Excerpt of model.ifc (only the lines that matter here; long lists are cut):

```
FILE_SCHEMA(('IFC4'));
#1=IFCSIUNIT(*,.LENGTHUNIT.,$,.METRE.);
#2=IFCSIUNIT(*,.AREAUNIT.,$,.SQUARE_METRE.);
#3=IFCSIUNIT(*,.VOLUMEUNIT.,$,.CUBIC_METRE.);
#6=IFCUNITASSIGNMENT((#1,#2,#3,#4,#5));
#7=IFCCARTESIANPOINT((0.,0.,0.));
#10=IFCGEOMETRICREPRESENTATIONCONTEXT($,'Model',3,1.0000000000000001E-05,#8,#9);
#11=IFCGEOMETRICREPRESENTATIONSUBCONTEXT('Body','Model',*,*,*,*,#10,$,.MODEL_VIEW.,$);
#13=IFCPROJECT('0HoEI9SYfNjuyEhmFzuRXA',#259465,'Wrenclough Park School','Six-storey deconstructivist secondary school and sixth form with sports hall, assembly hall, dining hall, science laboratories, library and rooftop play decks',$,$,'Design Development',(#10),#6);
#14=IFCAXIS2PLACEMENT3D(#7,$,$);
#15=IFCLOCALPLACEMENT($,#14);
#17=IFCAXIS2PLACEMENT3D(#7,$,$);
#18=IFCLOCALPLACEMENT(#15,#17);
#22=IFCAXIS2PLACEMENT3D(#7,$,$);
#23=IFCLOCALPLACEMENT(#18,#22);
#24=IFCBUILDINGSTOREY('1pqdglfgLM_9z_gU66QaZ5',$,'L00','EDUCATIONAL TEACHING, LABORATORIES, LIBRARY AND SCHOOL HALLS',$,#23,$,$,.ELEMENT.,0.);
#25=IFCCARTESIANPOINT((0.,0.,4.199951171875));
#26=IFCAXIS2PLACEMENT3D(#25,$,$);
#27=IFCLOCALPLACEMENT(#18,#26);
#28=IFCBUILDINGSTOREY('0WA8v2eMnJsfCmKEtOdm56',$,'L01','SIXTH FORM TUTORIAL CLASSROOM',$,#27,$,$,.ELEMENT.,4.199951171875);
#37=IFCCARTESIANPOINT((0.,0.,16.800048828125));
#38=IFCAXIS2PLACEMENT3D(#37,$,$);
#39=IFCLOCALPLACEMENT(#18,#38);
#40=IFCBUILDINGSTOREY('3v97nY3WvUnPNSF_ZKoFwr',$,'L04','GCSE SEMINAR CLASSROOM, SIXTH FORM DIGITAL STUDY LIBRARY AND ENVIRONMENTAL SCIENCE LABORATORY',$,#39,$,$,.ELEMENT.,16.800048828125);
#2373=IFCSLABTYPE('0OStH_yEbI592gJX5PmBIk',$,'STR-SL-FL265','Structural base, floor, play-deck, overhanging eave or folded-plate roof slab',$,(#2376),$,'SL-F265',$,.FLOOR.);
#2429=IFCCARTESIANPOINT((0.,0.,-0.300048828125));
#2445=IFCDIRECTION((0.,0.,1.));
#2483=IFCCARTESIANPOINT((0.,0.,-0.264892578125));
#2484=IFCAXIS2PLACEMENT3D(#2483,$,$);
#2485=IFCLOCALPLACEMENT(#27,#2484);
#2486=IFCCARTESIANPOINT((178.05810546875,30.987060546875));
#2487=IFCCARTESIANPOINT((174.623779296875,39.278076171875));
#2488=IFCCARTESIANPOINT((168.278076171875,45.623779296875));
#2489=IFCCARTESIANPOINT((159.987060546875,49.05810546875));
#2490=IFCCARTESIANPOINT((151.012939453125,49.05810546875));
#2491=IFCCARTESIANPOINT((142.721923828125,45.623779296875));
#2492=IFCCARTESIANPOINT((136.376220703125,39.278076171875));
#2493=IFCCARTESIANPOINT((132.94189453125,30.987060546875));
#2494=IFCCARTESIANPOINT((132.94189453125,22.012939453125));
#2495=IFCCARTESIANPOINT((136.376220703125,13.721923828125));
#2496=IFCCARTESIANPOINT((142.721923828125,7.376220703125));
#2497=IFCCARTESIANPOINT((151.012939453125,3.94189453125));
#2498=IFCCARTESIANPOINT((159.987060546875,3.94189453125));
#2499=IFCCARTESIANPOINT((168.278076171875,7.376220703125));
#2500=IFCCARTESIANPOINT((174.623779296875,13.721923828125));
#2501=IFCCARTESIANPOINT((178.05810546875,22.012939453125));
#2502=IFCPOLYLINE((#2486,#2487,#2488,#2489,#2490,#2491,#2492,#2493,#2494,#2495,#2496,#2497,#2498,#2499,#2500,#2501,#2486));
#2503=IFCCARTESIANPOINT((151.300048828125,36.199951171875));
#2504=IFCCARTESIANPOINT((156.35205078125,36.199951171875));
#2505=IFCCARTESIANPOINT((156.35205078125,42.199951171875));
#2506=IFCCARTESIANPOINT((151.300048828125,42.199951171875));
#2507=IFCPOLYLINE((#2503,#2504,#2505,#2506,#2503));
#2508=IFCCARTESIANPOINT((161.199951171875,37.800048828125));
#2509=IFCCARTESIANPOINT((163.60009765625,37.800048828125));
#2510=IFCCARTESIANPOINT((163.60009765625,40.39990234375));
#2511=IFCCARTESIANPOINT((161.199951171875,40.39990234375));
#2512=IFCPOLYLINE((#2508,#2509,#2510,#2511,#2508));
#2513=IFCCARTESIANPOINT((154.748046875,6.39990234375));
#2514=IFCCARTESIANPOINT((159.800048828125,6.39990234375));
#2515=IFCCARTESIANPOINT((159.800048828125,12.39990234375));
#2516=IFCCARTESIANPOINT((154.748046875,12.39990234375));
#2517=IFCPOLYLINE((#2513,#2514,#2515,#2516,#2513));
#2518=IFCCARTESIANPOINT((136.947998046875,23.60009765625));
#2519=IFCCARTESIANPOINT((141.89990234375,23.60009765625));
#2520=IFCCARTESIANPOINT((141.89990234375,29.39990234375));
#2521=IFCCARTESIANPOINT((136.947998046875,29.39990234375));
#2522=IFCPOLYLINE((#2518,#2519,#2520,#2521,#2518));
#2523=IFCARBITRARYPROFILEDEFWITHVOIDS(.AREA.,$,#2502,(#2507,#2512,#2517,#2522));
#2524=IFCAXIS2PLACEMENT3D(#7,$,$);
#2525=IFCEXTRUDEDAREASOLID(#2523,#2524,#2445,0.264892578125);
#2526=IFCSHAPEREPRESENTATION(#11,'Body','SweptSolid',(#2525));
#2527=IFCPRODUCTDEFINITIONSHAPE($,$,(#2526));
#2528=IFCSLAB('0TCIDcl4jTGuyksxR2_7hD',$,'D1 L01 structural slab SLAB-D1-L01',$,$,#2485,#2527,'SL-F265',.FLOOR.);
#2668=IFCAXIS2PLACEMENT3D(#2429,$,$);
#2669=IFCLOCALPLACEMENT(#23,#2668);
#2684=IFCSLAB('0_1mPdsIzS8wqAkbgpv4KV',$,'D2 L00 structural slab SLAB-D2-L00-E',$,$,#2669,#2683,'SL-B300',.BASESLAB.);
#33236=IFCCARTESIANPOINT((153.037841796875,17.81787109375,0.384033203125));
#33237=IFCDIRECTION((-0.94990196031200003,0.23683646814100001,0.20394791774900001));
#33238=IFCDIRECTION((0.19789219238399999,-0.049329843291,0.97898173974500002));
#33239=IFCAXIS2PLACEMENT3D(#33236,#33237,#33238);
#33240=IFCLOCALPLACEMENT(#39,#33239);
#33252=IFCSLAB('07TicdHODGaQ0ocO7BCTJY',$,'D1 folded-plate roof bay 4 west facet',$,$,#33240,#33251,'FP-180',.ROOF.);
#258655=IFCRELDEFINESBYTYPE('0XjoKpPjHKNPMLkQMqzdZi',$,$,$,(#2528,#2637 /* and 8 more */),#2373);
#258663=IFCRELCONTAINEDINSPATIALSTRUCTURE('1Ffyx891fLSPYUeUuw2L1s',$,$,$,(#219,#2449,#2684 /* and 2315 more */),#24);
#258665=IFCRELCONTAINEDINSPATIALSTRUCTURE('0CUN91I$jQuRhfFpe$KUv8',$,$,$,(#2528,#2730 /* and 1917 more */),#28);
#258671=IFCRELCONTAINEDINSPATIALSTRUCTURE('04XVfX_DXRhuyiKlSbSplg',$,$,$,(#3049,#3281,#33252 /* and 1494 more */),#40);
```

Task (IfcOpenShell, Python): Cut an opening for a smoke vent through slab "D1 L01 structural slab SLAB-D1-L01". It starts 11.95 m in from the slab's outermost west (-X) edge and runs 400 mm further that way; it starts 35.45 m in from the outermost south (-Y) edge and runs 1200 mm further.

```python
import numpy as np
import ifcopenshell
import ifcopenshell.api.feature
import ifcopenshell.api.geometry
import ifcopenshell.api.root
import ifcopenshell.geom
import ifcopenshell.util.placement
import ifcopenshell.util.representation
import ifcopenshell.util.shape
import ifcopenshell.util.unit

model = ifcopenshell.open("model.ifc")
unit_scale = ifcopenshell.util.unit.calculate_unit_scale(model)
settings = ifcopenshell.geom.settings()


def volume(element):
    """Net volume in cubic metres, openings subtracted."""
    shape = ifcopenshell.geom.create_shape(settings, element)
    return ifcopenshell.util.shape.get_volume(shape.geometry)


slab = model.by_guid("0TCIDcl4jTGuyksxR2_7hD")
before = volume(slab)

# Extent in the slab's own axes, in metres. The edges named are its -X and -Y sides.
slab_shape = ifcopenshell.geom.create_shape(settings, slab)
vertices = ifcopenshell.util.shape.get_vertices(slab_shape.geometry)
x_min, y_min, bottom = vertices.min(axis=0)
top = vertices[:, 2].max()

opening = ifcopenshell.api.root.create_entity(model, ifc_class="IfcOpeningElement", name="Smoke vent opening", predefined_type="OPENING")
context = ifcopenshell.util.representation.get_context(model, "Model", "Body", "MODEL_VIEW")
width, depth = 0.4, 1.2
outline = [(0.0, 0.0), (width, 0.0), (width, depth), (0.0, depth), (0.0, 0.0)]
# Overshoot both faces by 50 mm so the cut is clean.
shape = ifcopenshell.api.geometry.add_slab_representation(
    model, context=context, depth=top - bottom + 0.1, polyline=outline
)
ifcopenshell.api.geometry.assign_representation(model, product=opening, representation=shape)

matrix = ifcopenshell.util.placement.get_local_placement(slab.ObjectPlacement)
matrix[:, 3] = matrix @ np.append(np.array([x_min + 11.95, y_min + 35.45, bottom - 0.05]) / unit_scale, 1.0)
ifcopenshell.api.geometry.edit_object_placement(model, product=opening, matrix=matrix, is_si=False)
ifcopenshell.api.feature.add_feature(model, feature=opening, element=slab)

after = volume(slab)

print(f"slab volume {before:.3f} -> {after:.3f} m3")

model.write("model_updated.ifc")
```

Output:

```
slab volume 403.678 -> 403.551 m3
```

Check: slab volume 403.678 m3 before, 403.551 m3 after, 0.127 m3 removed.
